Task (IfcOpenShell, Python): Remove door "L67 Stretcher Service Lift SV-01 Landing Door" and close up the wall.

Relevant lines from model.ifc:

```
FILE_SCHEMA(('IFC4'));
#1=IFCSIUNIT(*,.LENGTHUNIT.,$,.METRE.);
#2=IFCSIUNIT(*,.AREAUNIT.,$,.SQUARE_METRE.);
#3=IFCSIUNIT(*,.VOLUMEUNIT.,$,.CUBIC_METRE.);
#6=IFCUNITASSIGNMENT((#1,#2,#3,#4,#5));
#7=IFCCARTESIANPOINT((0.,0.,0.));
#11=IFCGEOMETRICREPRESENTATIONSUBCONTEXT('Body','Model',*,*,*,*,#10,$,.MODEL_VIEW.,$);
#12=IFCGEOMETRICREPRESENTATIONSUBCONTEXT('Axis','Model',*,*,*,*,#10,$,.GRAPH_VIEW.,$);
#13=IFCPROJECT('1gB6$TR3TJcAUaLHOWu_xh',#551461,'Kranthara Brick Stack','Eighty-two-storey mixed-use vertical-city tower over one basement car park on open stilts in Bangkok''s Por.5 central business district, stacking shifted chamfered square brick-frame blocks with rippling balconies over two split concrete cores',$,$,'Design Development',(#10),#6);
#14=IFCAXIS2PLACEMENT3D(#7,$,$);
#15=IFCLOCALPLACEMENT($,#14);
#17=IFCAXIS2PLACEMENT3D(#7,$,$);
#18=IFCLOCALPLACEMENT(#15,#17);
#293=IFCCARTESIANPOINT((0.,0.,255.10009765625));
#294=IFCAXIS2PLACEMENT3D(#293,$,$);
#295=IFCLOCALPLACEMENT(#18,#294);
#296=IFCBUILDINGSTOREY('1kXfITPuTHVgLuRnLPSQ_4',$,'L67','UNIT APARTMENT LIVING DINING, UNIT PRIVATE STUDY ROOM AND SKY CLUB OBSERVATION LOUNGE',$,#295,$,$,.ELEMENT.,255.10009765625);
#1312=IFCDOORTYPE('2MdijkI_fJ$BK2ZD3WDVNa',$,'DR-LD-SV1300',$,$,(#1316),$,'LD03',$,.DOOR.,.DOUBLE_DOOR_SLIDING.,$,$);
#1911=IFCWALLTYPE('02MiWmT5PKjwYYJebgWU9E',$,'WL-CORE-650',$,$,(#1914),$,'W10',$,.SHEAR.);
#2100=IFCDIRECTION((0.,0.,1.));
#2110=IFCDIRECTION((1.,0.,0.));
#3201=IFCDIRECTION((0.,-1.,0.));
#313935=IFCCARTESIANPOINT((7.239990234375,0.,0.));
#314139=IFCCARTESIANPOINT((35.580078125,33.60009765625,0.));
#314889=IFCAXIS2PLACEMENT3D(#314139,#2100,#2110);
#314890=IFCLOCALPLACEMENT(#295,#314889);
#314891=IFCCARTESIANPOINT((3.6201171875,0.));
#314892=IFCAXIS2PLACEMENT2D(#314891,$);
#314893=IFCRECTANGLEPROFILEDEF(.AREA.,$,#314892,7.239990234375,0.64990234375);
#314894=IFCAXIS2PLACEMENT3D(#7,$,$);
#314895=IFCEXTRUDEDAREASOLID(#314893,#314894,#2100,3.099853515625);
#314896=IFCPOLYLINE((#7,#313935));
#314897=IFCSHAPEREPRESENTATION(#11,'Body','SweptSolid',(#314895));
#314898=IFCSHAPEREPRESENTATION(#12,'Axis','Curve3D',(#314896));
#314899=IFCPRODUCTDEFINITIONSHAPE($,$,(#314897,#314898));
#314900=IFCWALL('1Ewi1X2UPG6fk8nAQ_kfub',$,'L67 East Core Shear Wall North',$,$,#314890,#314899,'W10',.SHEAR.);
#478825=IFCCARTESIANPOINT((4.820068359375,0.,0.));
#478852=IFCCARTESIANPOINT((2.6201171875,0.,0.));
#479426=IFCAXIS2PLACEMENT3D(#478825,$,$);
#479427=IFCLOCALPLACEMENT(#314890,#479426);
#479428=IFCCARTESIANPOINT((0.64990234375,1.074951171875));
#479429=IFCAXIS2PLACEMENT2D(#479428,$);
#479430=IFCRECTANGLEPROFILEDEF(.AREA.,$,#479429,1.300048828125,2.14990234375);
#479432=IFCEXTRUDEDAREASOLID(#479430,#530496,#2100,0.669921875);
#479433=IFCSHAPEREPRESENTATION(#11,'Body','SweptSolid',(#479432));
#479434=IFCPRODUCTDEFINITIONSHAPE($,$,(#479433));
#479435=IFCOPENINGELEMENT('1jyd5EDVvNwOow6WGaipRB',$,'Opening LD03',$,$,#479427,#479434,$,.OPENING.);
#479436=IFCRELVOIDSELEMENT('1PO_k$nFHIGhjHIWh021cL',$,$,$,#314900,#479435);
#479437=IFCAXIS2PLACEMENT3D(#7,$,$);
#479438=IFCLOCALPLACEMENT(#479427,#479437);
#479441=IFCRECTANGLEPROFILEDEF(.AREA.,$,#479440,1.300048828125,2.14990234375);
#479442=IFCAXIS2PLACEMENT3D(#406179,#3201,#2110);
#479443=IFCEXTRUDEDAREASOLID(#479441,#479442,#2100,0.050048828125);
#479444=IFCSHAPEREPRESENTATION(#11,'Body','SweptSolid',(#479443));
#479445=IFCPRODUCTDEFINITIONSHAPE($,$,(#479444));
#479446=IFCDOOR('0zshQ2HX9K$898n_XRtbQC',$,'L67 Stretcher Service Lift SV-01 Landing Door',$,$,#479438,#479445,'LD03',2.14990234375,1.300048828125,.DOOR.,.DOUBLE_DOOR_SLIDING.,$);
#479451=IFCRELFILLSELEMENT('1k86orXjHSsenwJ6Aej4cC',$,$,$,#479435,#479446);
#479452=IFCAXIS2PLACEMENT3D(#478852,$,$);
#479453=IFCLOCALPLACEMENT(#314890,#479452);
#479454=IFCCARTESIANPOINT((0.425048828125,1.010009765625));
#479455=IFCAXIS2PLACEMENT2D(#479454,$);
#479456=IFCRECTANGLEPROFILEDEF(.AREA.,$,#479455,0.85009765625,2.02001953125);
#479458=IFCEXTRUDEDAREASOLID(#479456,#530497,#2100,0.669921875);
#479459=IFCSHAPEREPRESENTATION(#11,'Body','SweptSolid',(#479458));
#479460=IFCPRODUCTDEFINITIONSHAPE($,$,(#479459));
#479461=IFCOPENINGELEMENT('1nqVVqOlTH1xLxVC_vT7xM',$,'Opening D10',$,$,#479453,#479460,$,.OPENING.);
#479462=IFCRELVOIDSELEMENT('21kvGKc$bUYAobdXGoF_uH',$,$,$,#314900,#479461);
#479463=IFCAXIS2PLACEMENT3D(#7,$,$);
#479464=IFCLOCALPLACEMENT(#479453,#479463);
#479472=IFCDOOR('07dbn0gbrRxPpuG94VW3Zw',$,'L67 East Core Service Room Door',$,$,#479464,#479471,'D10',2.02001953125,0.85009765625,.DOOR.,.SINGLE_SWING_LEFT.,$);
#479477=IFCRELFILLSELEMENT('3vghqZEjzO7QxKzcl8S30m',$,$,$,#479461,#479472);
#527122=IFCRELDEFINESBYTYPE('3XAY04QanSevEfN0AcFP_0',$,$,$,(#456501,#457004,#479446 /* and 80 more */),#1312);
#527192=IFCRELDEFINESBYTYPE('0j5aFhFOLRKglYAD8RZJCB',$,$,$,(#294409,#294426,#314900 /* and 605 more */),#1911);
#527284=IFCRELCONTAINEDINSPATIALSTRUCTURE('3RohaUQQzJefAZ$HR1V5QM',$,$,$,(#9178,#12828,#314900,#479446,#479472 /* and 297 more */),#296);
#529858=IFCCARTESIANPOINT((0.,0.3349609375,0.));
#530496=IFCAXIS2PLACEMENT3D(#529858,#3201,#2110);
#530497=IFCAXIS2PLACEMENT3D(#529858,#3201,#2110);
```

```python
import ifcopenshell
import ifcopenshell.api.feature
import ifcopenshell.api.root
import ifcopenshell.geom
import ifcopenshell.util.shape

model = ifcopenshell.open("model.ifc")
settings = ifcopenshell.geom.settings()


def volume(element):
    """Net volume in cubic metres, openings subtracted."""
    shape = ifcopenshell.geom.create_shape(settings, element)
    return ifcopenshell.util.shape.get_volume(shape.geometry)


door = model.by_guid("0zshQ2HX9K$898n_XRtbQC")
opening = door.FillsVoids[0].RelatingOpeningElement
wall = opening.VoidsElements[0].RelatingBuildingElement
before = volume(wall)

ifcopenshell.api.root.remove_product(model, product=door)
ifcopenshell.api.feature.remove_feature(model, feature=opening)

after = volume(wall)

print(f"wall volume {before:.3f} -> {after:.3f} m3")

model.write("model-out.ifc")
```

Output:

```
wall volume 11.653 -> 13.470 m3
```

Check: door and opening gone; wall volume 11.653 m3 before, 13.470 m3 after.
